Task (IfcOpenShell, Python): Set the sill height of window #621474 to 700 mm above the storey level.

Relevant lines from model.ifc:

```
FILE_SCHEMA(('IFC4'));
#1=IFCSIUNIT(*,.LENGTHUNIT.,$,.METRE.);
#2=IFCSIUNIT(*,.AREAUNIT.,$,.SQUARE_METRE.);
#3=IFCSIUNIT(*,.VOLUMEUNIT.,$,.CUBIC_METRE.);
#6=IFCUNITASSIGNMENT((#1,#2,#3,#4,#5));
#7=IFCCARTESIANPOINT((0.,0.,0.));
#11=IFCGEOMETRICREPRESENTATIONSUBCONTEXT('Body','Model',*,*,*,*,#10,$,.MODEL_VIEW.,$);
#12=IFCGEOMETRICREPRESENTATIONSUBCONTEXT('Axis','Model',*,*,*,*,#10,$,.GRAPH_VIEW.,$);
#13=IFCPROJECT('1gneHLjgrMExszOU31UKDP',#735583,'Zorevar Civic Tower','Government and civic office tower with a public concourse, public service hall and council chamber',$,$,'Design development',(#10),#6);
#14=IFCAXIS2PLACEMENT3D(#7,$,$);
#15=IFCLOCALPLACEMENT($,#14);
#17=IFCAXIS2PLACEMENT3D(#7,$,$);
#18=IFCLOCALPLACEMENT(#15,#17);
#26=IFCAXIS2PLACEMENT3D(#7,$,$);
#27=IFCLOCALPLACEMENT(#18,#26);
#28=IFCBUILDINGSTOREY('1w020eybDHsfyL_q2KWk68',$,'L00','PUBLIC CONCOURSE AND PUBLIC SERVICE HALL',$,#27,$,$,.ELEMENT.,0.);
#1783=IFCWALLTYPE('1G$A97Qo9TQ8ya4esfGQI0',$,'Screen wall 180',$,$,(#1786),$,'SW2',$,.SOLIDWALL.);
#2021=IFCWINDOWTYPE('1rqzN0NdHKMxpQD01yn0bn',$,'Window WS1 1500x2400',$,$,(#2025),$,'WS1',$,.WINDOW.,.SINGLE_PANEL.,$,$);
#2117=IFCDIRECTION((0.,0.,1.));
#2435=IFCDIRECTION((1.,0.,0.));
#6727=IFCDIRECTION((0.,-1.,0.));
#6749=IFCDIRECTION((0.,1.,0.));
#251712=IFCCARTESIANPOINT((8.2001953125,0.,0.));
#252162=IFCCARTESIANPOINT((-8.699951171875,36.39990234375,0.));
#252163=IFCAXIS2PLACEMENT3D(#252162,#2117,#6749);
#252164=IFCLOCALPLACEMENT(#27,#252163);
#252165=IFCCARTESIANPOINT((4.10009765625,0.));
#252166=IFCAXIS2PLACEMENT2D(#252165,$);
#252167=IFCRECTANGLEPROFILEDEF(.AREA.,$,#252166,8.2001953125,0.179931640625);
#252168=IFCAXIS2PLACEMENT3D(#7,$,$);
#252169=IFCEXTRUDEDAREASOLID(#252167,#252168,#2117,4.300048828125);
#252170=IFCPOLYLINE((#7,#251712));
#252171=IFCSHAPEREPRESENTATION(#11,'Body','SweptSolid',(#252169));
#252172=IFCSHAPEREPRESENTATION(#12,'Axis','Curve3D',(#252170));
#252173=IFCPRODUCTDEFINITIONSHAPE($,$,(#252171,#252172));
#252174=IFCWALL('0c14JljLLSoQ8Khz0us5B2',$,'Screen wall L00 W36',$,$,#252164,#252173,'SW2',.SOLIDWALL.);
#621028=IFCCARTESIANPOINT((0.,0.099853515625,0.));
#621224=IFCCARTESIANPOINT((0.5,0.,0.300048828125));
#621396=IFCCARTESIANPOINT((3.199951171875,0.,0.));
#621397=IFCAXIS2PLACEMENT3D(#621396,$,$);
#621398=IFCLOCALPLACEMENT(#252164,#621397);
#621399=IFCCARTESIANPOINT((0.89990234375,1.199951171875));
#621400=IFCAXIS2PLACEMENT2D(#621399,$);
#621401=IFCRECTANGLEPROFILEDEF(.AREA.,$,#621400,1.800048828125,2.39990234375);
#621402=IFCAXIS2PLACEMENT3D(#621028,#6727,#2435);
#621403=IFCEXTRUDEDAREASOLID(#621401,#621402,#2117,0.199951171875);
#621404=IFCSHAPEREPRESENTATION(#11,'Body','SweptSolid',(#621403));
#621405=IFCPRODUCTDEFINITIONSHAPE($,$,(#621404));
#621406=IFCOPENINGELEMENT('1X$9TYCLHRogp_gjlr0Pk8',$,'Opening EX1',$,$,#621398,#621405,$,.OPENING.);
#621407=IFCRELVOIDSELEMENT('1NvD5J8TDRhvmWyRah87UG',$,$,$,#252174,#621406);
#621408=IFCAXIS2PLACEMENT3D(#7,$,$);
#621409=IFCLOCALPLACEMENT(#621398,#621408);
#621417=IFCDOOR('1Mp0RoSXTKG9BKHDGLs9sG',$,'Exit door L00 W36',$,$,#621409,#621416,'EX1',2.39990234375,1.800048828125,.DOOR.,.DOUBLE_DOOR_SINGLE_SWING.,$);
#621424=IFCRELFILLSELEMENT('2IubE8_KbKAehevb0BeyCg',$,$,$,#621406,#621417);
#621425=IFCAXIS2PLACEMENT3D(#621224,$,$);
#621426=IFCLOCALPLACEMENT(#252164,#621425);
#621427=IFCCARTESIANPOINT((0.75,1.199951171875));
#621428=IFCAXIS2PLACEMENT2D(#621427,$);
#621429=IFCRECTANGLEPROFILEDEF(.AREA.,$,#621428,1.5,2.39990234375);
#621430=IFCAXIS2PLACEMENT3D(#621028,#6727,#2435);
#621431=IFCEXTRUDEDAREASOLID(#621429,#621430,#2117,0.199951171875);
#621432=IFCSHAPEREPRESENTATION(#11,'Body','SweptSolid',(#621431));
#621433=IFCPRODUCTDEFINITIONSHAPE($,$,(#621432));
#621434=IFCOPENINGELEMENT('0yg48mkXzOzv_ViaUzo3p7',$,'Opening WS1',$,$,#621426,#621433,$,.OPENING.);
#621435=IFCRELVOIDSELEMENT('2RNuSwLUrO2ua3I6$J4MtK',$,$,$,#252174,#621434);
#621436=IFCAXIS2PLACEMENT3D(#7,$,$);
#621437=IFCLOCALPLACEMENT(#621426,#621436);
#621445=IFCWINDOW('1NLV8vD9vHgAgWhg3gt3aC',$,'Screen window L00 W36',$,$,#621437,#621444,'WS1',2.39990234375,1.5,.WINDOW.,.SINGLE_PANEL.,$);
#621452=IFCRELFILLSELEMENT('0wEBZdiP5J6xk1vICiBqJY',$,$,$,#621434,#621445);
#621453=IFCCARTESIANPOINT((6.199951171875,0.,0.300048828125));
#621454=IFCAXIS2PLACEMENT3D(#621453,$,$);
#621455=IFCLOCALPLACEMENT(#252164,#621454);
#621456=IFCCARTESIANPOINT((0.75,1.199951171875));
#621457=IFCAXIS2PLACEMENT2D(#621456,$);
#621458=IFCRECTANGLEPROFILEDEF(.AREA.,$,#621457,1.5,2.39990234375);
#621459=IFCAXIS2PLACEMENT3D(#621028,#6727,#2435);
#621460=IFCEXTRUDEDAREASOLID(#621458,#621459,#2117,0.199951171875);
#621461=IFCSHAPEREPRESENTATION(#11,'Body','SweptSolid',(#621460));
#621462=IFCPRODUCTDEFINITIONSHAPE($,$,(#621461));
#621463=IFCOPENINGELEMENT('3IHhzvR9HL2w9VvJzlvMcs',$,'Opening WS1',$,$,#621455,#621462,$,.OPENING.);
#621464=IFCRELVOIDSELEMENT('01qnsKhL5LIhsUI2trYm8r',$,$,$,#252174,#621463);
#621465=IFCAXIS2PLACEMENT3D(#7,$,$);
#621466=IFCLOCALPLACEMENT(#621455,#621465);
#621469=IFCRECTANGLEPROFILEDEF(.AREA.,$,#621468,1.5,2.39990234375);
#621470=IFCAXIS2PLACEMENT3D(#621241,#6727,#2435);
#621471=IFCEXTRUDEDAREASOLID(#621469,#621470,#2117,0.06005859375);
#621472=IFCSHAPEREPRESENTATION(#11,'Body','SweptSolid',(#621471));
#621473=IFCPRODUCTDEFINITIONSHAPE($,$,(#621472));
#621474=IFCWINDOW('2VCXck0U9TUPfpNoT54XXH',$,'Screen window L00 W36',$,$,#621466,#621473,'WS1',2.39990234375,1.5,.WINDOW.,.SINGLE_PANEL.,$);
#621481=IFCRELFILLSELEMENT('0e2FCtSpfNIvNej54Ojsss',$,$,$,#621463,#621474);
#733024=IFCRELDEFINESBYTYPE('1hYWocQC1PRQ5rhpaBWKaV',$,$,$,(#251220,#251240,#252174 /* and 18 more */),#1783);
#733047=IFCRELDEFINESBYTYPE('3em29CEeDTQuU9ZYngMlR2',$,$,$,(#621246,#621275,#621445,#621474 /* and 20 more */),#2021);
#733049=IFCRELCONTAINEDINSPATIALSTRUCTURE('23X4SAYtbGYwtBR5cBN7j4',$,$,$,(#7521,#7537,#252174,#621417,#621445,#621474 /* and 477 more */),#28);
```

```python
import numpy as np
import ifcopenshell
import ifcopenshell.api.geometry
import ifcopenshell.geom
import ifcopenshell.util.element
import ifcopenshell.util.placement
import ifcopenshell.util.shape
import ifcopenshell.util.unit

model = ifcopenshell.open("model.ifc")
unit_scale = ifcopenshell.util.unit.calculate_unit_scale(model)

window = model.by_guid("2VCXck0U9TUPfpNoT54XXH")
opening = window.FillsVoids[0].RelatingOpeningElement
storey = ifcopenshell.util.element.get_container(window, ifc_class="IfcBuildingStorey")
level = ifcopenshell.util.placement.get_local_placement(storey.ObjectPlacement)[2, 3]

# The opening's origin need not be at the sill, so measure its lowest point.
shape = ifcopenshell.geom.create_shape(ifcopenshell.geom.settings(), opening)
bottom = ifcopenshell.util.shape.get_shape_bottom_elevation(shape, shape.geometry) / unit_scale
dz = level + 0.7 / unit_scale - bottom

shift = np.array([0.0, 0.0, dz])
# The window is placed relative to its opening, so it follows when the opening moves.
matrix = ifcopenshell.util.placement.get_local_placement(opening.ObjectPlacement)
matrix[:3, 3] += shift
ifcopenshell.api.geometry.edit_object_placement(
    model, product=opening, matrix=matrix, is_si=False, should_transform_children=True
)

print(f"moved by {dz * unit_scale:+.3f} m")

model.write("model_updated.ifc")
```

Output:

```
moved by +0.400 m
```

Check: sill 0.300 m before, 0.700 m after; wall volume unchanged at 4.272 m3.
